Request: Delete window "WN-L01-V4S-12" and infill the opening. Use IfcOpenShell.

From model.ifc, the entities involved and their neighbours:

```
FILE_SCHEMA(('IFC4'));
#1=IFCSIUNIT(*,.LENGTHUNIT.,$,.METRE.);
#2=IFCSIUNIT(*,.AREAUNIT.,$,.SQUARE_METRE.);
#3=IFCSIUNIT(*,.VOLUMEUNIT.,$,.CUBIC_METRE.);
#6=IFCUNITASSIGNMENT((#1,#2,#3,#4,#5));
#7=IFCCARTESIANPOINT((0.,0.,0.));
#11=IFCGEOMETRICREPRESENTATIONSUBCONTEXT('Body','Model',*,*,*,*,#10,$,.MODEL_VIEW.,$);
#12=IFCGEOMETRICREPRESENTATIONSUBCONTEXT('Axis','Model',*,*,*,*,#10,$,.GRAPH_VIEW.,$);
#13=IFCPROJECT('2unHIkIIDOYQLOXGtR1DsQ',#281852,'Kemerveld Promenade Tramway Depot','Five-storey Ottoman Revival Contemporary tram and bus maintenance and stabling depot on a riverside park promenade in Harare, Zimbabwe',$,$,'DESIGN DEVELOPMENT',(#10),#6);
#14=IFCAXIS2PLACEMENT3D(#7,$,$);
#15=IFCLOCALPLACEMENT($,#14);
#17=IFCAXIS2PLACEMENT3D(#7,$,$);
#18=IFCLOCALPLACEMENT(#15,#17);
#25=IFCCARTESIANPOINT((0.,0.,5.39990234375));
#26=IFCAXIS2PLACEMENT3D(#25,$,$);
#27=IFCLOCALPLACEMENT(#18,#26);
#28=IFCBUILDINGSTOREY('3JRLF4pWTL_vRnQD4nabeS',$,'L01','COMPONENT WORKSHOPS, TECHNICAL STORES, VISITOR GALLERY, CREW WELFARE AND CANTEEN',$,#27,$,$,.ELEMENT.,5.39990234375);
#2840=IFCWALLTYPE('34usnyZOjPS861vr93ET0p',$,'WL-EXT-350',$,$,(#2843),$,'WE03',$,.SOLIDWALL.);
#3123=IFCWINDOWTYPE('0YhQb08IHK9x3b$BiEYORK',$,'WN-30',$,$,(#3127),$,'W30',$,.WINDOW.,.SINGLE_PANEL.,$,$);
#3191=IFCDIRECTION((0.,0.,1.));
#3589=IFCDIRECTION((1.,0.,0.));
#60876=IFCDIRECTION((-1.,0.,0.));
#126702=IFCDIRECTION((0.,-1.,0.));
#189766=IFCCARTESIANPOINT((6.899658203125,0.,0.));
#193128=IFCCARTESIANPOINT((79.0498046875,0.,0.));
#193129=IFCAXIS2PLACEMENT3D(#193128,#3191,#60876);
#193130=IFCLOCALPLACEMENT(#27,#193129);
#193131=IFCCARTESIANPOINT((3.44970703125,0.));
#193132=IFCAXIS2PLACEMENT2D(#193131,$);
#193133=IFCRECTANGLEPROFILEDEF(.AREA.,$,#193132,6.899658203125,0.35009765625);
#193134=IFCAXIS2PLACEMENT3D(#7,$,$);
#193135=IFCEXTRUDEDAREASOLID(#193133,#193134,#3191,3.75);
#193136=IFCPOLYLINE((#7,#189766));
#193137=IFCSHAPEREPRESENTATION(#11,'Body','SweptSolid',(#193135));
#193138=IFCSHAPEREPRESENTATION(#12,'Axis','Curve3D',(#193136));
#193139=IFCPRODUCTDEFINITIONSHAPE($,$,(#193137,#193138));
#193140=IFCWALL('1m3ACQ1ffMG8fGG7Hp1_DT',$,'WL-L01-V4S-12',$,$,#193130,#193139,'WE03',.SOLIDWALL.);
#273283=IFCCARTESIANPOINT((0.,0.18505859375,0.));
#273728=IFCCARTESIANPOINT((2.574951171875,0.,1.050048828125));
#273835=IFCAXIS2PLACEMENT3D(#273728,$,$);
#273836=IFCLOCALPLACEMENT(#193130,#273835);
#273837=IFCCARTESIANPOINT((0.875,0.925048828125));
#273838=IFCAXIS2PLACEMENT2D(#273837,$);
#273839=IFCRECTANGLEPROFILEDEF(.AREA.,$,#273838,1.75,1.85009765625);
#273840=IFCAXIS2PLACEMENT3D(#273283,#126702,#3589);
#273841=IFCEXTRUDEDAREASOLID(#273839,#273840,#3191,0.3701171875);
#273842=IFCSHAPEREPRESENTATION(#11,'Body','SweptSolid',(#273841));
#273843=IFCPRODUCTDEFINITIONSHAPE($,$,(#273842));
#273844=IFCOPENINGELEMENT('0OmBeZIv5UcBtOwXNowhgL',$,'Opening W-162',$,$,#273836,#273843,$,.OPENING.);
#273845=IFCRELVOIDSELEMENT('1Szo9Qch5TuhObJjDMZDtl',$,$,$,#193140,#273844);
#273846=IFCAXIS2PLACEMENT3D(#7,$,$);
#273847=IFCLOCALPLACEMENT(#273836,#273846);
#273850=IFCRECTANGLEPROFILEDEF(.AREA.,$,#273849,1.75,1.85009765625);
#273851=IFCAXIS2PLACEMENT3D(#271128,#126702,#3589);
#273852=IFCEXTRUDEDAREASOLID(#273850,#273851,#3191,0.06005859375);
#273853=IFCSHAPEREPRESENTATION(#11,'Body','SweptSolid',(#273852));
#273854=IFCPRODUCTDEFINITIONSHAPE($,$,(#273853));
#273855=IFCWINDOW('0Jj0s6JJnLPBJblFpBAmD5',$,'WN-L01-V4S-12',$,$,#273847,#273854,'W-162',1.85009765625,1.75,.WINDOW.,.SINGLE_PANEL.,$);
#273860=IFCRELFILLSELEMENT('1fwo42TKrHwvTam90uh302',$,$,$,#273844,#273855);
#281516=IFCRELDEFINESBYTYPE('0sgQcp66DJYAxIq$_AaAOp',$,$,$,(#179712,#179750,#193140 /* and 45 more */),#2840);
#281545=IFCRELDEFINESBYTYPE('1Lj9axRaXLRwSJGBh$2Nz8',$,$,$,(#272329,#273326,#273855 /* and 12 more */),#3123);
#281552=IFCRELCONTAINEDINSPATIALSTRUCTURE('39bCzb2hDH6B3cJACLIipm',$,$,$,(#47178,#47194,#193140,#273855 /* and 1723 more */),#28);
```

```python
import ifcopenshell
import ifcopenshell.api.feature
import ifcopenshell.api.root
import ifcopenshell.geom
import ifcopenshell.util.shape

model = ifcopenshell.open("model.ifc")
settings = ifcopenshell.geom.settings()


def volume(element):
    """Net volume in cubic metres, openings subtracted."""
    shape = ifcopenshell.geom.create_shape(settings, element)
    return ifcopenshell.util.shape.get_volume(shape.geometry)


window = model.by_guid("0Jj0s6JJnLPBJblFpBAmD5")
opening = window.FillsVoids[0].RelatingOpeningElement
wall = opening.VoidsElements[0].RelatingBuildingElement
before = volume(wall)

ifcopenshell.api.root.remove_product(model, product=window)
ifcopenshell.api.feature.remove_feature(model, feature=opening)

after = volume(wall)

print(f"wall volume {before:.3f} -> {after:.3f} m3")

model.write("model_rev.ifc")
```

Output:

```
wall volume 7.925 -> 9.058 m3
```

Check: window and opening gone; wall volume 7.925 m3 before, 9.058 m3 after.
